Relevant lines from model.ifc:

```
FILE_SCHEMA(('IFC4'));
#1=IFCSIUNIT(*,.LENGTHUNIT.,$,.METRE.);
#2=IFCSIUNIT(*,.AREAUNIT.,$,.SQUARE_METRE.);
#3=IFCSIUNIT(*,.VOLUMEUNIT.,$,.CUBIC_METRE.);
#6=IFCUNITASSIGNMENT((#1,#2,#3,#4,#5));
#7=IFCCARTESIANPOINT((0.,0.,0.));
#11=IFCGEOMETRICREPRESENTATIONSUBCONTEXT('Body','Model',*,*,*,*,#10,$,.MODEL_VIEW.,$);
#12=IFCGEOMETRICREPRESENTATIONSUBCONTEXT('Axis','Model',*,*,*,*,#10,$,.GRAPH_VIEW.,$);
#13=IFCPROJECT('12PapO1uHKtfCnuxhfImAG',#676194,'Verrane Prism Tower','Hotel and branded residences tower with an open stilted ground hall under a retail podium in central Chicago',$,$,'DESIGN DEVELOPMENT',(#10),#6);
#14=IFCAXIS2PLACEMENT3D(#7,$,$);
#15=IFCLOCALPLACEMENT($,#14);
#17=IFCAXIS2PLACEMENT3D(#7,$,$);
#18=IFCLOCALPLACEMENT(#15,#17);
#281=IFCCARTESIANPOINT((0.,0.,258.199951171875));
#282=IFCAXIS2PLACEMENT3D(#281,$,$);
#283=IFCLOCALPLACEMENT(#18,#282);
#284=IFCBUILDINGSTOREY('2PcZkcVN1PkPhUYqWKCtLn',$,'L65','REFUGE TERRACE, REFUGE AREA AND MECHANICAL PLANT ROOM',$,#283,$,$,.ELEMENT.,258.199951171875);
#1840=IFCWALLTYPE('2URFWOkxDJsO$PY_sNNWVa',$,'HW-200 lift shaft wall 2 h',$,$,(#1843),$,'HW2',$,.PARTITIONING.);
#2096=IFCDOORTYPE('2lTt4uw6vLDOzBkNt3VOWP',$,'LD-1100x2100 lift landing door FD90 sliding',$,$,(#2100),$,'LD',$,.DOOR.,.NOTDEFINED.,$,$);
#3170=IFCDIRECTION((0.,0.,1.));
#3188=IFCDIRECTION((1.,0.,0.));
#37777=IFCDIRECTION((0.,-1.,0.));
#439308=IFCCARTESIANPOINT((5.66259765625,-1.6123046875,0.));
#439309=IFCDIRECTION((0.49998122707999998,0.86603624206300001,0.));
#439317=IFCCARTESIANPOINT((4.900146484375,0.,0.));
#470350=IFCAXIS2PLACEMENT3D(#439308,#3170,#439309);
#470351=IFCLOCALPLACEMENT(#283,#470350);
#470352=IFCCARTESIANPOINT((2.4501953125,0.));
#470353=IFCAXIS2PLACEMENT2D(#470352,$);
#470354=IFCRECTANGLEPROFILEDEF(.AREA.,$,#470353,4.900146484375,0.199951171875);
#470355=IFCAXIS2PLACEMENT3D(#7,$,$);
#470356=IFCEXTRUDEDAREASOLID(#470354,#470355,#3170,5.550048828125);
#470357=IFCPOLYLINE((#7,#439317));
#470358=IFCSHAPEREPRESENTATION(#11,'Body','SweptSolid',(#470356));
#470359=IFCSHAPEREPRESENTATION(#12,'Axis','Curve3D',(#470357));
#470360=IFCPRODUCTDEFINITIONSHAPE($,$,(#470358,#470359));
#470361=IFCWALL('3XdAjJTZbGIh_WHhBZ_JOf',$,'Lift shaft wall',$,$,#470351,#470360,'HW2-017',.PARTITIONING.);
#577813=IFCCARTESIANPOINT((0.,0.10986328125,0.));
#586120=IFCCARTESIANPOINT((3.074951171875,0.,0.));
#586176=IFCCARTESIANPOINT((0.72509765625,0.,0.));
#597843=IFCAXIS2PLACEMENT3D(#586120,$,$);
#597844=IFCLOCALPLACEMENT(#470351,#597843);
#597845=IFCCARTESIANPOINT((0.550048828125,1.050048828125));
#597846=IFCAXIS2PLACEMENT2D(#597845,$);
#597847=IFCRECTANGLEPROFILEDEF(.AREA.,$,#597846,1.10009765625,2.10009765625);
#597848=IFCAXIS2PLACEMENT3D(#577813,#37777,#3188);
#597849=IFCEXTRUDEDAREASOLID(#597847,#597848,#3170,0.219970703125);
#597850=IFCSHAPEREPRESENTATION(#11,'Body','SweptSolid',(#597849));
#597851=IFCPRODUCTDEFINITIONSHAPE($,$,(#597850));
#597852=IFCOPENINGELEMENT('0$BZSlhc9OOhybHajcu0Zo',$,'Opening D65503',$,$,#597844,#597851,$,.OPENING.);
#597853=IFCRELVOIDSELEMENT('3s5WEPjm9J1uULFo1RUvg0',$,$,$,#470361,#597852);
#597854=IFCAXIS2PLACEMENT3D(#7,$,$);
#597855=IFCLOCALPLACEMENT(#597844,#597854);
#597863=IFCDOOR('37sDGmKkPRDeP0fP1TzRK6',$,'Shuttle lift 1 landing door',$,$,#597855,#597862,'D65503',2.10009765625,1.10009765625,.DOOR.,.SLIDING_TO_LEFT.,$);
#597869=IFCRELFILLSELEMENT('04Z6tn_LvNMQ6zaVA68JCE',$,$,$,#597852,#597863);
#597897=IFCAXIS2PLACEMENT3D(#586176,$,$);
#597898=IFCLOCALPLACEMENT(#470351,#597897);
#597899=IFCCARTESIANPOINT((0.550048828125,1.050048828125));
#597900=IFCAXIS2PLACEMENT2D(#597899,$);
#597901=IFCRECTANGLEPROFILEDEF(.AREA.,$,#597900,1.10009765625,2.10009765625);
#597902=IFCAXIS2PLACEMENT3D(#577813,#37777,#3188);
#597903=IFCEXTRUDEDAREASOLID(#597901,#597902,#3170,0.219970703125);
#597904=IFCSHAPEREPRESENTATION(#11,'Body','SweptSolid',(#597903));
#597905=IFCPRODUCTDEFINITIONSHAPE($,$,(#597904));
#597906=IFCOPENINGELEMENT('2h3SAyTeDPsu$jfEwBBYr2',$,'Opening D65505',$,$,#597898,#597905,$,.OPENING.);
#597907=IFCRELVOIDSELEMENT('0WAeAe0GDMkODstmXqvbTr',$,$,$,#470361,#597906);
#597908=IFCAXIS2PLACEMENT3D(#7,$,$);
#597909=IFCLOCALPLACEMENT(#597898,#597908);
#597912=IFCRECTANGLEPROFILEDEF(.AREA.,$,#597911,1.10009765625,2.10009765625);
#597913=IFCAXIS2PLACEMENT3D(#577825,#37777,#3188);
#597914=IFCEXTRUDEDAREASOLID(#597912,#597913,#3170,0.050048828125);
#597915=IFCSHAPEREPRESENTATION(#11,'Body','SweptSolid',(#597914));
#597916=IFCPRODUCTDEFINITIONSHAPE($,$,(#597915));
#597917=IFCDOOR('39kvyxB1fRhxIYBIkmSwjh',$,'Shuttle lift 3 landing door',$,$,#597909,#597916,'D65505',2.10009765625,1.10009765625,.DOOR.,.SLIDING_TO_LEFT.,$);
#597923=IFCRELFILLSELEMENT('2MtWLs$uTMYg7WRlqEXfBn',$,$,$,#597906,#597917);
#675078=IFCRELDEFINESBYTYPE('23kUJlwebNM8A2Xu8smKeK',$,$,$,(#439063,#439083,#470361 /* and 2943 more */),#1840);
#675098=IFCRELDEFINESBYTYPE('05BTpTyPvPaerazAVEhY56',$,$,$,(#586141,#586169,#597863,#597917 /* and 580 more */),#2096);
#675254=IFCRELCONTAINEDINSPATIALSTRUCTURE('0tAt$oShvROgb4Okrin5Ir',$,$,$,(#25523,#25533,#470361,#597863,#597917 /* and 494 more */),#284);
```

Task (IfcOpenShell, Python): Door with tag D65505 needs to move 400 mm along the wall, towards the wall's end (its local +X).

```python
import ifcopenshell
import ifcopenshell.api.geometry
import ifcopenshell.util.placement

model = ifcopenshell.open("model.ifc")

door = model.by_guid("39kvyxB1fRhxIYBIkmSwjh")
opening = door.FillsVoids[0].RelatingOpeningElement
wall = opening.VoidsElements[0].RelatingBuildingElement

wall_matrix = ifcopenshell.util.placement.get_local_placement(wall.ObjectPlacement)
shift = wall_matrix[:3, 0] * 0.4
before = ifcopenshell.util.placement.get_local_placement(door.ObjectPlacement)[:3, 3].copy()

# The door is placed relative to its opening, so it follows when the opening moves.
matrix = ifcopenshell.util.placement.get_local_placement(opening.ObjectPlacement)
matrix[:3, 3] += shift
ifcopenshell.api.geometry.edit_object_placement(
    model, product=opening, matrix=matrix, is_si=False, should_transform_children=True
)

after = ifcopenshell.util.placement.get_local_placement(door.ObjectPlacement)[:3, 3]
print("door moved by", (after - before).round(3) + 0.0)

model.write("model_rev.ifc")
```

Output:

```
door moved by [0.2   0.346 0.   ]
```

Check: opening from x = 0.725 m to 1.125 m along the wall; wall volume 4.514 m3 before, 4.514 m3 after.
